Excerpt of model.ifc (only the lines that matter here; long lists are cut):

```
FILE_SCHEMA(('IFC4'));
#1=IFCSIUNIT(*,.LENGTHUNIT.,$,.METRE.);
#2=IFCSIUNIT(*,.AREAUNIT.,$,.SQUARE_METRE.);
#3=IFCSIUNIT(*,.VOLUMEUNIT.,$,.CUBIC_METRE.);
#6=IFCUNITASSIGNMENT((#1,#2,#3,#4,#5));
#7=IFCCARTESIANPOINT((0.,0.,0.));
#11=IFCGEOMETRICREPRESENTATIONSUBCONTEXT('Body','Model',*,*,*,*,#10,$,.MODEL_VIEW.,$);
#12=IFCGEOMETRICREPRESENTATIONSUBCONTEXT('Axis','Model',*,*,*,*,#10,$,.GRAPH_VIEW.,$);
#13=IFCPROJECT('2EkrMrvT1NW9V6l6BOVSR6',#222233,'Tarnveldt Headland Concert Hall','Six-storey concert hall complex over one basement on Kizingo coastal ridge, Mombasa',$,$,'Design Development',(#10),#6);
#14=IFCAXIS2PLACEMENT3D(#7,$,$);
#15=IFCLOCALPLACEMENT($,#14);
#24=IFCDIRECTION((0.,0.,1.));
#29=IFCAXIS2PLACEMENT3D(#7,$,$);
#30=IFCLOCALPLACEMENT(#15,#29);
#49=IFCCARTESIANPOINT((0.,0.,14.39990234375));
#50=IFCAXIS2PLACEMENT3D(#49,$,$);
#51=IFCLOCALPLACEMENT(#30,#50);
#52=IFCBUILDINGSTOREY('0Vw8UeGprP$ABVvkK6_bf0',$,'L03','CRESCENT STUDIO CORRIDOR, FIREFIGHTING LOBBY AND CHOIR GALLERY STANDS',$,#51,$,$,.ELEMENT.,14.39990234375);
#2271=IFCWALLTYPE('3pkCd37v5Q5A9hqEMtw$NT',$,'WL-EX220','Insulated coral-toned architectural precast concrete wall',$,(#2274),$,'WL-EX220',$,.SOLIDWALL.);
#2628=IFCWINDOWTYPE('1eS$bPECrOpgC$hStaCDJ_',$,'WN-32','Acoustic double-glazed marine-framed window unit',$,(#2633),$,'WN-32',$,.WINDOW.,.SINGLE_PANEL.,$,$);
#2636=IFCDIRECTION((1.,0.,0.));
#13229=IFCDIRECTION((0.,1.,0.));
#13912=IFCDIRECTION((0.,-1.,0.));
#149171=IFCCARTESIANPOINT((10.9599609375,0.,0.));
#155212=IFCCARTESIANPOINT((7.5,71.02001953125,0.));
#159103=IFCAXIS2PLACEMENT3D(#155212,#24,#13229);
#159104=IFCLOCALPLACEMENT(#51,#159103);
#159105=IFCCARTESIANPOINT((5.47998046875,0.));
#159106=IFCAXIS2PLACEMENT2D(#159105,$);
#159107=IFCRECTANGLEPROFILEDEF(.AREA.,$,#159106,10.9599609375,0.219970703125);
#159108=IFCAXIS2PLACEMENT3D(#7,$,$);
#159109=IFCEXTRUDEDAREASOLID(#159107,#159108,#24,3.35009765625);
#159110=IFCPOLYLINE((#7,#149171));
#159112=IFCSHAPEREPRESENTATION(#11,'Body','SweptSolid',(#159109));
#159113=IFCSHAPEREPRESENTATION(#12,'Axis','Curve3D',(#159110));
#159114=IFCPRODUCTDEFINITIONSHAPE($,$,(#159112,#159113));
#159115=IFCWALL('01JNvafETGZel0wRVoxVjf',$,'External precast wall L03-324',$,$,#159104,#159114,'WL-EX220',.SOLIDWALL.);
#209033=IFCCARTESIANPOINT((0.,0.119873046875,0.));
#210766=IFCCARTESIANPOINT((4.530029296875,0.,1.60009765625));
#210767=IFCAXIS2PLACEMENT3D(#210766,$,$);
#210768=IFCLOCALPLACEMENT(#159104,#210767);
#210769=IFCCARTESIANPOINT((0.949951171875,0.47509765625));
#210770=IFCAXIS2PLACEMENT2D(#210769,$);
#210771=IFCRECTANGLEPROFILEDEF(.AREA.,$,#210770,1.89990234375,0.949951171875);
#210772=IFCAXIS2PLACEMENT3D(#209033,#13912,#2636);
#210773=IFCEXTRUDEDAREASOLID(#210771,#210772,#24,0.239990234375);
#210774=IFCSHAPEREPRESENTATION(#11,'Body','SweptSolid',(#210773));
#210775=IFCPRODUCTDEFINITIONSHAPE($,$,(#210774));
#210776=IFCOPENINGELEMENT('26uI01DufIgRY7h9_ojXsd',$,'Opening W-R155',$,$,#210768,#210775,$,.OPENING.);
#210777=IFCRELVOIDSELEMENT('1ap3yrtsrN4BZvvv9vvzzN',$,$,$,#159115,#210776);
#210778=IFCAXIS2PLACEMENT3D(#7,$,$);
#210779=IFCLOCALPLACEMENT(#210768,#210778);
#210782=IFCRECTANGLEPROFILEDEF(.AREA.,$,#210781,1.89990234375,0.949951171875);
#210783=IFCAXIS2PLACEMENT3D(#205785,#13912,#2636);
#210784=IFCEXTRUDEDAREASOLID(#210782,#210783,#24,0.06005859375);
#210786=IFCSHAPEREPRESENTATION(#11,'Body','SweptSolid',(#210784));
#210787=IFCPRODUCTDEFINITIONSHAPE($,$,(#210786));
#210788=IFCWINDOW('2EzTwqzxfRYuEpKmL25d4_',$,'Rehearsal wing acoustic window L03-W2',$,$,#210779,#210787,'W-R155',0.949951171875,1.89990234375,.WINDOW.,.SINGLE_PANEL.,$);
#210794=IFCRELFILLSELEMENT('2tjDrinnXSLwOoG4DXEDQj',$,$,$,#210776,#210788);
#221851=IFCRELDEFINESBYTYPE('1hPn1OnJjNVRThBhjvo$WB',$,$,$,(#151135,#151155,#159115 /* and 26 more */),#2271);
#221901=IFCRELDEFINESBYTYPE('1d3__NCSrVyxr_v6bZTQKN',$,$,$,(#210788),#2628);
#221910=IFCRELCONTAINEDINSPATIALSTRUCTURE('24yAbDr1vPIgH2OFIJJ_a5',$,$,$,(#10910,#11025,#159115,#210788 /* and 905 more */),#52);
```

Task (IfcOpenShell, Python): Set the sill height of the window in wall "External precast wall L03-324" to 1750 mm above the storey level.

```python
import numpy as np
import ifcopenshell
import ifcopenshell.api.geometry
import ifcopenshell.geom
import ifcopenshell.util.element
import ifcopenshell.util.placement
import ifcopenshell.util.shape
import ifcopenshell.util.unit

model = ifcopenshell.open("model.ifc")
unit_scale = ifcopenshell.util.unit.calculate_unit_scale(model)

window = model.by_id(210788)
opening = window.FillsVoids[0].RelatingOpeningElement
storey = ifcopenshell.util.element.get_container(window, ifc_class="IfcBuildingStorey")
level = ifcopenshell.util.placement.get_local_placement(storey.ObjectPlacement)[2, 3]

# The opening's origin need not be at the sill, so measure its lowest point.
shape = ifcopenshell.geom.create_shape(ifcopenshell.geom.settings(), opening)
bottom = ifcopenshell.util.shape.get_shape_bottom_elevation(shape, shape.geometry) / unit_scale
dz = level + 1.75 / unit_scale - bottom

shift = np.array([0.0, 0.0, dz])
# The window is placed relative to its opening, so it follows when the opening moves.
matrix = ifcopenshell.util.placement.get_local_placement(opening.ObjectPlacement)
matrix[:3, 3] += shift
ifcopenshell.api.geometry.edit_object_placement(
    model, product=opening, matrix=matrix, is_si=False, should_transform_children=True
)

print(f"moved by {dz * unit_scale:+.3f} m")

model.write("model_rev.ifc")
```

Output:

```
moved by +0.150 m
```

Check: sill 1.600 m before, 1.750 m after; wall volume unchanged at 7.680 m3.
